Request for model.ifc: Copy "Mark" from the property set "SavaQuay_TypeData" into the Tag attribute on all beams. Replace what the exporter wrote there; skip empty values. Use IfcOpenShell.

First a look at what the model holds.

```python
import ifcopenshell
import ifcopenshell.util.element

model = ifcopenshell.open("model.ifc")
print(model.schema)
beams = model.by_type("IfcBeam")
print(len(beams), "beams")
for e in beams[:8]:
    source = ifcopenshell.util.element.get_pset(e, "SavaQuay_TypeData", "Mark")
    target = e.Tag
    print(e.id(), repr(source), repr(target), sep=" | ")
```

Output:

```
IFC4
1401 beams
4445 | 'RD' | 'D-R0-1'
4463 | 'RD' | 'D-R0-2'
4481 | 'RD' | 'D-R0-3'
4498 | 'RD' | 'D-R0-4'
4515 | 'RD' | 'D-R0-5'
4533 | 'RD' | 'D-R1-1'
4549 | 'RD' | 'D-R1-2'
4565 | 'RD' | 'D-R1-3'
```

```python
import ifcopenshell
import ifcopenshell.util.element

model = ifcopenshell.open("model.ifc")

count = 0
for e in model.by_type("IfcBeam"):
    value = ifcopenshell.util.element.get_pset(e, "SavaQuay_TypeData", "Mark")
    current = e.Tag
    if not value or not value.strip() or current == value:
        continue
    e.Tag = value
    count += 1

print(count, "beams updated")

model.write("model_updated.ifc")
```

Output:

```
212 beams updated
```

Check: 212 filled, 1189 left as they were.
